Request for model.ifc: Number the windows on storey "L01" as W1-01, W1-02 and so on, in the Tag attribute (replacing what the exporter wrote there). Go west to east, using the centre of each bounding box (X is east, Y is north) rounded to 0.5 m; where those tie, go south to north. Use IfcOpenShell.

First a look at what the model holds.

```python
import ifcopenshell
import ifcopenshell.util.element
import ifcopenshell.util.placement

model = ifcopenshell.open("model.ifc")
print(model.schema)
storey = next(s for s in model.by_type("IfcBuildingStorey") if s.Name == "L01")
windows = [e for e in ifcopenshell.util.element.get_decomposition(storey) if e.is_a("IfcWindow")]
for e in sorted(windows, key=lambda e: e.id()):
    origin = ifcopenshell.util.placement.get_local_placement(e.ObjectPlacement)[:3, 3]
    print(e.id(), e.Tag, e.Name, origin.round(2) + 0.0, sep=" | ")
```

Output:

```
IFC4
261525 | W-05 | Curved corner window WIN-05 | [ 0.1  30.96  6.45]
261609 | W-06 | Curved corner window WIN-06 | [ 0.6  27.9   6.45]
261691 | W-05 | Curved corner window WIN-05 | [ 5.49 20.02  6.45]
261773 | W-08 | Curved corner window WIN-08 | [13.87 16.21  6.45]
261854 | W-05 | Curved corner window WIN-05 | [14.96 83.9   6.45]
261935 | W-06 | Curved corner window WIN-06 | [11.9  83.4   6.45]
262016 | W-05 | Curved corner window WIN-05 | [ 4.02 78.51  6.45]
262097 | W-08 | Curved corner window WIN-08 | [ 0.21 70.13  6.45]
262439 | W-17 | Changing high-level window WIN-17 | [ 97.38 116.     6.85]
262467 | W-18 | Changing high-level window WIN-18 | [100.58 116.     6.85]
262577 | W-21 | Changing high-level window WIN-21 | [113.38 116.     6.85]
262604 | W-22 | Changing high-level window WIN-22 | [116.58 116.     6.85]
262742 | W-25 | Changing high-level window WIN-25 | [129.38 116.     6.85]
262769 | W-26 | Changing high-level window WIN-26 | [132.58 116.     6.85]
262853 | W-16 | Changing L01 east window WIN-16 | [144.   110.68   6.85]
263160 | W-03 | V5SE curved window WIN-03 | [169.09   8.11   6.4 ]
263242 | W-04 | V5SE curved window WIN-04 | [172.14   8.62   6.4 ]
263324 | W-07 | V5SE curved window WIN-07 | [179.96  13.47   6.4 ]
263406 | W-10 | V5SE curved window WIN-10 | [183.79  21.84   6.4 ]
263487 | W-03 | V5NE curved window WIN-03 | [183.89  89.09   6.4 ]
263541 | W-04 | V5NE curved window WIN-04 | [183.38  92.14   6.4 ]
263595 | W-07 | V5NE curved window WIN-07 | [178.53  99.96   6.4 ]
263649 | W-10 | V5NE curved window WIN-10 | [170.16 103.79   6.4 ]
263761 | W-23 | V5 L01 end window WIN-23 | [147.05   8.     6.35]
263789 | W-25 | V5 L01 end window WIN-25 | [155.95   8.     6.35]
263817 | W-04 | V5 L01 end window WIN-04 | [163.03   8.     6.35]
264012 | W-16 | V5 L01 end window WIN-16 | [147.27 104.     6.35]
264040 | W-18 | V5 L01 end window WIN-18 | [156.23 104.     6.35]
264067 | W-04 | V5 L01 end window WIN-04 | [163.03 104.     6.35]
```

```python
import ifcopenshell
import ifcopenshell.geom
import ifcopenshell.util.element
import ifcopenshell.util.shape

model = ifcopenshell.open("model.ifc")
settings = ifcopenshell.geom.settings()
settings.set("use-world-coords", True)


def centre(element):
    shape = ifcopenshell.geom.create_shape(settings, element)
    return ifcopenshell.util.shape.get_bbox_centroid(shape.geometry)


storey = next(s for s in model.by_type("IfcBuildingStorey") if s.Name == "L01")
windows = [e for e in ifcopenshell.util.element.get_decomposition(storey) if e.is_a("IfcWindow")]

# Insertion points can sit at a corner or the storey origin, so sort by the geometry (in metres).
centres = {e: centre(e) for e in windows}
windows.sort(key=lambda e: (round(centres[e][0] / 0.5), centres[e][1]))

for i, e in enumerate(windows, start=1):
    number = f"W1-{i:02d}"
    e.Tag = number
    print(e.id(), number)

model.write("model_v2.ifc")
```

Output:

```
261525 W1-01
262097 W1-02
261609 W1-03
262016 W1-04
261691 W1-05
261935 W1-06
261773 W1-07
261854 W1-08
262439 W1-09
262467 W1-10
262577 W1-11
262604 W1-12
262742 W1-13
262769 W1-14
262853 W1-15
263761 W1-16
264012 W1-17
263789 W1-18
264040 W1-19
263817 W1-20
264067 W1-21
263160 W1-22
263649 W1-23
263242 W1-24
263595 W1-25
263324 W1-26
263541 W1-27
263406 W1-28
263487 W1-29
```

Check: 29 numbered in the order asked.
